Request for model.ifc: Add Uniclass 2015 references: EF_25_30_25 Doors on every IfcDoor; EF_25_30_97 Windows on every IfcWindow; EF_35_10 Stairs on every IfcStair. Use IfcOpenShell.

First a look at what the model holds.

```python
import ifcopenshell

model = ifcopenshell.open("model.ifc")
print(model.schema)
print("classifications:", [c.Name for c in model.by_type("IfcClassification")])
for ifc_class in ("IfcDoor", "IfcRoof", "IfcStair", "IfcWall", "IfcWindow"):
    print(ifc_class, len(model.by_type(ifc_class)))
```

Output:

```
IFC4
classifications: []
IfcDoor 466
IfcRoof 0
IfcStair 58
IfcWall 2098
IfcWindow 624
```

```python
import ifcopenshell
import ifcopenshell.api.classification

model = ifcopenshell.open("model.ifc")

system = ifcopenshell.api.classification.add_classification(model, classification="Uniclass 2015")

codes = {
    "IfcDoor": ("EF_25_30_25", "Doors"),
    "IfcWindow": ("EF_25_30_97", "Windows"),
    "IfcStair": ("EF_35_10", "Stairs"),
}
for ifc_class, (code, name) in codes.items():
    products = model.by_type(ifc_class)
    ifcopenshell.api.classification.add_reference(
        model, products=products, classification=system, identification=code, name=name
    )
    print(code, len(products))

model.write("model_updated.ifc")
```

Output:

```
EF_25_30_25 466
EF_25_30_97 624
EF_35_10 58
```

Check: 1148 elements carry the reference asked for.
